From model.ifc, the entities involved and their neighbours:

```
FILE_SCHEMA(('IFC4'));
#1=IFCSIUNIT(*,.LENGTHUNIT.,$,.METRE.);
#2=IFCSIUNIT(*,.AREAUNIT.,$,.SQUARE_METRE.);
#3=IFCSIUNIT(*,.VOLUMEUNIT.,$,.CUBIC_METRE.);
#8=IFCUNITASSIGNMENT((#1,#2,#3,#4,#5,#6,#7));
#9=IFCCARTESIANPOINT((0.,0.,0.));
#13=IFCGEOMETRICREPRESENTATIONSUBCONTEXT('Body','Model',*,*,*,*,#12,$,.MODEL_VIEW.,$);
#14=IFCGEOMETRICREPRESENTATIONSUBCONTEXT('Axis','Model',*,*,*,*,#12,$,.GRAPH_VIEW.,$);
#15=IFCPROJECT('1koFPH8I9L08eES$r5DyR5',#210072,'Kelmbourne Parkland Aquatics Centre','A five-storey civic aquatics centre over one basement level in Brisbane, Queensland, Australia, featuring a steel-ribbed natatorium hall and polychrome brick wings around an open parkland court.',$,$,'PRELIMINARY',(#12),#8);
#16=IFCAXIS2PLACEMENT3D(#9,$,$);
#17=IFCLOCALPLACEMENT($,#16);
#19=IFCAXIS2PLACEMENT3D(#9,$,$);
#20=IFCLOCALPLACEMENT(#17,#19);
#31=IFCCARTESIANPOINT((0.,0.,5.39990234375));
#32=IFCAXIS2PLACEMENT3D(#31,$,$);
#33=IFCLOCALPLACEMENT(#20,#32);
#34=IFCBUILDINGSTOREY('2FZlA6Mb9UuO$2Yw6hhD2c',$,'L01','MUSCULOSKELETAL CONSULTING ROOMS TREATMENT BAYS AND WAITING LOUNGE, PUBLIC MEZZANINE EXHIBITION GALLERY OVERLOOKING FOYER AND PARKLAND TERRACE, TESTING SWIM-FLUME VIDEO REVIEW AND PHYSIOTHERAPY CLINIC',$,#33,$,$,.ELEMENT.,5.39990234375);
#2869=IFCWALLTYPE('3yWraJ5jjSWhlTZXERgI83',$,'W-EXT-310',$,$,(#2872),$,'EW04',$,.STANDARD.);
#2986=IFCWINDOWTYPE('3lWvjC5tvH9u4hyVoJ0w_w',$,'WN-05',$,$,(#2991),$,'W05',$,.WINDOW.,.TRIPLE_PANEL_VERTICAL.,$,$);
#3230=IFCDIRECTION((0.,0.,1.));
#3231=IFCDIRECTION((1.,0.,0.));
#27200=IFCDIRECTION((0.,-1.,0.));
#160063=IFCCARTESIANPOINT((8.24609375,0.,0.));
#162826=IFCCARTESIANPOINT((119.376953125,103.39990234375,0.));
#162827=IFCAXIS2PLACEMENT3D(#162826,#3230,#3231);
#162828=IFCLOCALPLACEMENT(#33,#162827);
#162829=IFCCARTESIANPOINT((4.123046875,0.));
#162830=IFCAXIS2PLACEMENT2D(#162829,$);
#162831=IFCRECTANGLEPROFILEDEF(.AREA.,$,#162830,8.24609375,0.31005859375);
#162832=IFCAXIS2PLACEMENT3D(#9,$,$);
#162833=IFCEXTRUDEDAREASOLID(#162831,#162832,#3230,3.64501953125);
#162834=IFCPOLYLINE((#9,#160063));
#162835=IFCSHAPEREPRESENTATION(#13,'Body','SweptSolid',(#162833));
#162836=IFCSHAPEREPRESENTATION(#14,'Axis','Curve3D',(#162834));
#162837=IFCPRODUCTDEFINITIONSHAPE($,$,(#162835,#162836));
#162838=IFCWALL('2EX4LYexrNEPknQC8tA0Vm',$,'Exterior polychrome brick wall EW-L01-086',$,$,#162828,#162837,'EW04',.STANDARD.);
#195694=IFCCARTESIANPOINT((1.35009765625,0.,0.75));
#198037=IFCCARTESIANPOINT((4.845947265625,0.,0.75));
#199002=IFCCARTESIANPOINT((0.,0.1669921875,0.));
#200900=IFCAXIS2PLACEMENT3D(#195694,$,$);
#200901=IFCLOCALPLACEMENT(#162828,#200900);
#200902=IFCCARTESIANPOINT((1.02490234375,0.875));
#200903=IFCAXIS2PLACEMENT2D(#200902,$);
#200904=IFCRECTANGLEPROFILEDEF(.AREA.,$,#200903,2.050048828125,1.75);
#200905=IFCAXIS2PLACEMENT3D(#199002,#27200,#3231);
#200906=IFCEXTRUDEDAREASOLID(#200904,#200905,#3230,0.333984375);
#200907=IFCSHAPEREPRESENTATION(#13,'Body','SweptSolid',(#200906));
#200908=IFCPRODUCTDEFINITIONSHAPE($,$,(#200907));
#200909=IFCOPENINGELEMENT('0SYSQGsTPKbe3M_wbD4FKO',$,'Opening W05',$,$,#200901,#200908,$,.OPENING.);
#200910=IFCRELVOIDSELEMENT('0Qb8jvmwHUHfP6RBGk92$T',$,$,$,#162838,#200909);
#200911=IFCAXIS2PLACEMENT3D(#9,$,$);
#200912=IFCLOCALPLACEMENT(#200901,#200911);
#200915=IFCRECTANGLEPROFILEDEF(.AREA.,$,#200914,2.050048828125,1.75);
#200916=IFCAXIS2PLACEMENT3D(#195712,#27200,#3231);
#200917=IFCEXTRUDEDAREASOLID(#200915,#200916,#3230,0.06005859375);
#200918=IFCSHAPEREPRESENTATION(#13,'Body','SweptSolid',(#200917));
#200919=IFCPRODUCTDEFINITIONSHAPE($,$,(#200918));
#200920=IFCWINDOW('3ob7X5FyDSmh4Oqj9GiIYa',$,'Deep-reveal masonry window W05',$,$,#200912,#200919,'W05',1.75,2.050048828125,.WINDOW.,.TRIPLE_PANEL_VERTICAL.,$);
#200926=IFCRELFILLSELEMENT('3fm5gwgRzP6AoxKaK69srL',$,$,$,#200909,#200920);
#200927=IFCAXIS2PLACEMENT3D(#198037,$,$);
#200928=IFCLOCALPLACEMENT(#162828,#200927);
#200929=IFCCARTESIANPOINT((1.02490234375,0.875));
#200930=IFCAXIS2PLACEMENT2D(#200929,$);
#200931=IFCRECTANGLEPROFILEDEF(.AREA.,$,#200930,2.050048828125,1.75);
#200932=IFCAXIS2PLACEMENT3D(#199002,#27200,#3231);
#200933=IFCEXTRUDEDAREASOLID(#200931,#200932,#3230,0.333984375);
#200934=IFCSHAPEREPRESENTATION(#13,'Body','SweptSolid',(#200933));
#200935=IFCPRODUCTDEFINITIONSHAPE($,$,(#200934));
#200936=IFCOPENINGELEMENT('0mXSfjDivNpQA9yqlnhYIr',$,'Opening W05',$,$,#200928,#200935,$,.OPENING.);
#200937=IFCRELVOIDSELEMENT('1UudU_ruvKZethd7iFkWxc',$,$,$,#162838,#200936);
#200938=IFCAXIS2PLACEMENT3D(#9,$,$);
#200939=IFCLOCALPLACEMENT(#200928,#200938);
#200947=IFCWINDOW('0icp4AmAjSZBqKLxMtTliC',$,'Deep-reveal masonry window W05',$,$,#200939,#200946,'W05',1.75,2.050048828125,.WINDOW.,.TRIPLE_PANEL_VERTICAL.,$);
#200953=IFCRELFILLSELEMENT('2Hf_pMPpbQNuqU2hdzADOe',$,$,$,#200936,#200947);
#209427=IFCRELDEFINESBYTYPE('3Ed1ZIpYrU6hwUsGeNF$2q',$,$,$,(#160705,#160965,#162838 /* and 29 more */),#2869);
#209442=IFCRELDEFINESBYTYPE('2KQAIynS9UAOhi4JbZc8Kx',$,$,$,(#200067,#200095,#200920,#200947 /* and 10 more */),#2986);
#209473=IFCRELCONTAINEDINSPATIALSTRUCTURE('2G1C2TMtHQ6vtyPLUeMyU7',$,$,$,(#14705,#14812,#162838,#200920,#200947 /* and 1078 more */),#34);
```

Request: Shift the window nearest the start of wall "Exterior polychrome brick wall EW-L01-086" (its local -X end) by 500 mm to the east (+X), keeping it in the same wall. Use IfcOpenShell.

```python
import ifcopenshell
import ifcopenshell.api.geometry
import ifcopenshell.util.placement

model = ifcopenshell.open("model.ifc")

window = model.by_guid("3ob7X5FyDSmh4Oqj9GiIYa")
opening = window.FillsVoids[0].RelatingOpeningElement
wall = opening.VoidsElements[0].RelatingBuildingElement

wall_matrix = ifcopenshell.util.placement.get_local_placement(wall.ObjectPlacement)
shift = wall_matrix[:3, 0] * 0.5
before = ifcopenshell.util.placement.get_local_placement(window.ObjectPlacement)[:3, 3].copy()

# The window is placed relative to its opening, so it follows when the opening moves.
matrix = ifcopenshell.util.placement.get_local_placement(opening.ObjectPlacement)
matrix[:3, 3] += shift
ifcopenshell.api.geometry.edit_object_placement(
    model, product=opening, matrix=matrix, is_si=False, should_transform_children=True
)

after = ifcopenshell.util.placement.get_local_placement(window.ObjectPlacement)[:3, 3]
print("window moved by", (after - before).round(3) + 0.0)

model.write("model_updated.ifc")
```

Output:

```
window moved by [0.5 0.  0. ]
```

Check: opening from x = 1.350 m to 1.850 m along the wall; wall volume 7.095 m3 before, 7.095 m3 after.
